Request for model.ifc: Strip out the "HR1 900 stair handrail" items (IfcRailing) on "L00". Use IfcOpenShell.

First a look at what the model holds.

```python
import ifcopenshell
import ifcopenshell.util.element

model = ifcopenshell.open("model.ifc")
print(model.schema)
storey = next(s for s in model.by_type("IfcBuildingStorey") if s.Name == "L00")
railings = [e for e in ifcopenshell.util.element.get_decomposition(storey) if e.is_a("IfcRailing")]
seen = {}
for e in railings:
    element_type = ifcopenshell.util.element.get_type(e)
    name = element_type.Name if element_type not in (None, e) else None
    seen[name] = seen.get(name, 0) + 1
for name, count in sorted(seen.items(), key=str):
    print(count, "x", name)
```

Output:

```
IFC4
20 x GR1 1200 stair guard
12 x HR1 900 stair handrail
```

```python
import ifcopenshell
import ifcopenshell.api.root
import ifcopenshell.util.element

model = ifcopenshell.open("model.ifc")

storey = next(s for s in model.by_type("IfcBuildingStorey") if s.Name == "L00")
railings = [e for e in ifcopenshell.util.element.get_decomposition(storey) if e.is_a("IfcRailing")]
targets = [e for e in railings if (t := ifcopenshell.util.element.get_type(e)) not in (None, e) and t.Name == "HR1 900 stair handrail"]

for e in targets:
    ifcopenshell.api.root.remove_product(model, product=e)
print(len(targets), "removed")

model.write("model_edited.ifc")
```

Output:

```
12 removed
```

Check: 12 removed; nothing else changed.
